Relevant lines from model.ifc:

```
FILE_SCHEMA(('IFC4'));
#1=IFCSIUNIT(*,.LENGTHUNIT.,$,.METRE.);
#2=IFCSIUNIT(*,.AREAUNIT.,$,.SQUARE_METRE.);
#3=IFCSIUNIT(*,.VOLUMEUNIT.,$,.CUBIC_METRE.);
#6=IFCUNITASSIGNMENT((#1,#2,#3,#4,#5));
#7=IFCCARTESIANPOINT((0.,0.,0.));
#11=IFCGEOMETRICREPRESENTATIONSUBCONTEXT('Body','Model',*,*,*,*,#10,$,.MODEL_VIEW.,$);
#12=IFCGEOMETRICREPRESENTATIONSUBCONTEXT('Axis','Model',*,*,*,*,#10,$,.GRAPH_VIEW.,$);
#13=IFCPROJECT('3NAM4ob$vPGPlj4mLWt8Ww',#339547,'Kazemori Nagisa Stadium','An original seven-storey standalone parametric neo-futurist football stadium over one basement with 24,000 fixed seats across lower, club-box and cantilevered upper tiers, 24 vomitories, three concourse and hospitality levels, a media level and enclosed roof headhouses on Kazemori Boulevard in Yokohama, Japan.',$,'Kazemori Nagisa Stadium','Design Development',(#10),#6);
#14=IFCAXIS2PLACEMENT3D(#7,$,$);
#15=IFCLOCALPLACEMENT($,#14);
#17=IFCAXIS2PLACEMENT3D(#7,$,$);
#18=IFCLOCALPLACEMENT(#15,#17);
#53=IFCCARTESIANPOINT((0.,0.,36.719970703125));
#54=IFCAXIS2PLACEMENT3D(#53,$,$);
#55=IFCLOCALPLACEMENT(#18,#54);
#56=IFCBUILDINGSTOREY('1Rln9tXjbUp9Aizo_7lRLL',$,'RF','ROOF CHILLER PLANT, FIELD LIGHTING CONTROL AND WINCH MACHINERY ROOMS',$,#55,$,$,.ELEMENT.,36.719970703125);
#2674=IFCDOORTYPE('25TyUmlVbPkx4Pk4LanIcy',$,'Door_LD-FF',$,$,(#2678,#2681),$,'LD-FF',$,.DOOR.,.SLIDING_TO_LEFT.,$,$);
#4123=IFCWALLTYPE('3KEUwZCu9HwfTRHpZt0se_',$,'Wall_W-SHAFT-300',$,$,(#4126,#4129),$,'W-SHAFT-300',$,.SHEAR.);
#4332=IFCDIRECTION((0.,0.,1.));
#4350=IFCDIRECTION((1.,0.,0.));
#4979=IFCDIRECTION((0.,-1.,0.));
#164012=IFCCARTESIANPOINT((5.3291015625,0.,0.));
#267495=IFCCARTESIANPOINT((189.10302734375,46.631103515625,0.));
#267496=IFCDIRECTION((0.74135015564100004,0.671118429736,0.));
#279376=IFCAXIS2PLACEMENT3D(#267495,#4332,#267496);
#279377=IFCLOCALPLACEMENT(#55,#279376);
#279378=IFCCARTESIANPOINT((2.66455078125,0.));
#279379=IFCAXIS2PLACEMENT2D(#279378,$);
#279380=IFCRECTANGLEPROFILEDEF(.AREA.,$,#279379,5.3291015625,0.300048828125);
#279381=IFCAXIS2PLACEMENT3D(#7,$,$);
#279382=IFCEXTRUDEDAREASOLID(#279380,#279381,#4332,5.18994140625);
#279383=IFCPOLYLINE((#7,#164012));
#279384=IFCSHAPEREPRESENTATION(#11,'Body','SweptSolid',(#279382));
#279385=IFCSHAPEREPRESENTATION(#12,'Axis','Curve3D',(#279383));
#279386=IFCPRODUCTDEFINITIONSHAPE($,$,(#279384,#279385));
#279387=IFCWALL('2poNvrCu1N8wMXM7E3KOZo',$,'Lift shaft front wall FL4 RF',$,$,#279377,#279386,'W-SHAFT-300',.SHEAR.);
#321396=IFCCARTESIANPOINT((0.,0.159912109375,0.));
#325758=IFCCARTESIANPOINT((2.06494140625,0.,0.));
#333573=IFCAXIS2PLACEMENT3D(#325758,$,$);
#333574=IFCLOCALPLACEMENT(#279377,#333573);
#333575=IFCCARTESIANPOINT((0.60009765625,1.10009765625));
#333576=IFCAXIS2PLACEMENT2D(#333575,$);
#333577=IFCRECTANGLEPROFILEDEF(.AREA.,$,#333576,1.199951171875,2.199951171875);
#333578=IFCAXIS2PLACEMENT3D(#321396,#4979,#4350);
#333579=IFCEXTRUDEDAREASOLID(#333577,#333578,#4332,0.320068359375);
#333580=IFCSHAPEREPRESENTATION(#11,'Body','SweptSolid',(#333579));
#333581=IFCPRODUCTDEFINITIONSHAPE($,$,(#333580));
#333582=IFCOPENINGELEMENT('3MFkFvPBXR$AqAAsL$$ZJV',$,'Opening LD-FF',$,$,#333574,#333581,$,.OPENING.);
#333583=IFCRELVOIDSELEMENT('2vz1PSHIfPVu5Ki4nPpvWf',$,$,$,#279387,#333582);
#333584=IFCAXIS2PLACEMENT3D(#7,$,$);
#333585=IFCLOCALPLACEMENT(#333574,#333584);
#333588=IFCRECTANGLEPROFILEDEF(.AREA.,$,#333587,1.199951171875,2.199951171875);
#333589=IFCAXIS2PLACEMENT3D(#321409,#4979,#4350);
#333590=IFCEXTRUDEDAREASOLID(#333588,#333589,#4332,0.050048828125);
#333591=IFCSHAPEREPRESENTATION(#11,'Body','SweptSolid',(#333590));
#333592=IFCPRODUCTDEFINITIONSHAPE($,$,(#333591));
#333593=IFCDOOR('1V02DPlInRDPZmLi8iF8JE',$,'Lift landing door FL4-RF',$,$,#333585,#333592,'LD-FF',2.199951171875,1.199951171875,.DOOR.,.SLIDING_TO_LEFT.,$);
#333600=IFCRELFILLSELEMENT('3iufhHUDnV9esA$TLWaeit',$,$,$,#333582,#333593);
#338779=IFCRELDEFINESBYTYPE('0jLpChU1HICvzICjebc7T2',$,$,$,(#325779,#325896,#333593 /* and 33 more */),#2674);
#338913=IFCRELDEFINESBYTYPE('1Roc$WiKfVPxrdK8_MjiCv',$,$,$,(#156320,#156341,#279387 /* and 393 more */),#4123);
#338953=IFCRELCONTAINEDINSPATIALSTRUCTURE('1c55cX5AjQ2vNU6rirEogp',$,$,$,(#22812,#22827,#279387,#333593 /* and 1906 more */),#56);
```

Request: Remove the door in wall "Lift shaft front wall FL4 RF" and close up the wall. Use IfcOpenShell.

```python
import ifcopenshell
import ifcopenshell.api.feature
import ifcopenshell.api.root
import ifcopenshell.geom
import ifcopenshell.util.shape

model = ifcopenshell.open("model.ifc")
settings = ifcopenshell.geom.settings()


def volume(element):
    """Net volume in cubic metres, openings subtracted."""
    shape = ifcopenshell.geom.create_shape(settings, element)
    return ifcopenshell.util.shape.get_volume(shape.geometry)


door = model.by_guid("1V02DPlInRDPZmLi8iF8JE")
opening = door.FillsVoids[0].RelatingOpeningElement
wall = opening.VoidsElements[0].RelatingBuildingElement
before = volume(wall)

ifcopenshell.api.root.remove_product(model, product=door)
ifcopenshell.api.feature.remove_feature(model, feature=opening)

after = volume(wall)

print(f"wall volume {before:.3f} -> {after:.3f} m3")

model.write("model_rev.ifc")
```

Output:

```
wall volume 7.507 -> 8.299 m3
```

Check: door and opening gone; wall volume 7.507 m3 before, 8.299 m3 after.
